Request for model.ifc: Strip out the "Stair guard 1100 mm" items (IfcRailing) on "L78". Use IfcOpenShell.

First a look at what the model holds.

```python
import ifcopenshell
import ifcopenshell.util.element

model = ifcopenshell.open("model.ifc")
print(model.schema)
storey = next(s for s in model.by_type("IfcBuildingStorey") if s.Name == "L78")
railings = [e for e in ifcopenshell.util.element.get_decomposition(storey) if e.is_a("IfcRailing")]
seen = {}
for e in railings:
    element_type = ifcopenshell.util.element.get_type(e)
    name = element_type.Name if element_type not in (None, e) else None
    seen[name] = seen.get(name, 0) + 1
for name, count in sorted(seen.items(), key=str):
    print(count, "x", name)
```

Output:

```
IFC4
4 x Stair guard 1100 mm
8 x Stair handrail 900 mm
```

```python
import ifcopenshell
import ifcopenshell.api.root
import ifcopenshell.util.element

model = ifcopenshell.open("model.ifc")

storey = next(s for s in model.by_type("IfcBuildingStorey") if s.Name == "L78")
railings = [e for e in ifcopenshell.util.element.get_decomposition(storey) if e.is_a("IfcRailing")]
targets = [e for e in railings if (t := ifcopenshell.util.element.get_type(e)) not in (None, e) and t.Name == "Stair guard 1100 mm"]

for e in targets:
    ifcopenshell.api.root.remove_product(model, product=e)
print(len(targets), "removed")

model.write("model_rev.ifc")
```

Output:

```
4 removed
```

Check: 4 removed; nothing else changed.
